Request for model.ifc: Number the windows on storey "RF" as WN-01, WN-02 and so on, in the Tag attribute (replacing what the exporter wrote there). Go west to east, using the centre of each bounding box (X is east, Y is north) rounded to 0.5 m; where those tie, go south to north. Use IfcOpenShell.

First a look at what the model holds.

```python
import ifcopenshell
import ifcopenshell.util.element
import ifcopenshell.util.placement

model = ifcopenshell.open("model.ifc")
print(model.schema)
storey = next(s for s in model.by_type("IfcBuildingStorey") if s.Name == "RF")
windows = [e for e in ifcopenshell.util.element.get_decomposition(storey) if e.is_a("IfcWindow")]
for e in sorted(windows, key=lambda e: e.id()):
    origin = ifcopenshell.util.placement.get_local_placement(e.ObjectPlacement)[:3, 3]
    print(e.id(), e.Tag, e.Name, origin.round(2) + 0.0, sep=" | ")
```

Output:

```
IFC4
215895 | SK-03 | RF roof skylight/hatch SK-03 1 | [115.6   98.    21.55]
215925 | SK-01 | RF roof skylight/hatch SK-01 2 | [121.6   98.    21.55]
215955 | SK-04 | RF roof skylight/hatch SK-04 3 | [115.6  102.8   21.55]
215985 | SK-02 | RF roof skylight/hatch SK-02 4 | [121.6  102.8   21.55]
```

```python
import ifcopenshell
import ifcopenshell.geom
import ifcopenshell.util.element
import ifcopenshell.util.shape

model = ifcopenshell.open("model.ifc")
settings = ifcopenshell.geom.settings()
settings.set("use-world-coords", True)


def centre(element):
    shape = ifcopenshell.geom.create_shape(settings, element)
    return ifcopenshell.util.shape.get_bbox_centroid(shape.geometry)


storey = next(s for s in model.by_type("IfcBuildingStorey") if s.Name == "RF")
windows = [e for e in ifcopenshell.util.element.get_decomposition(storey) if e.is_a("IfcWindow")]

# Insertion points can sit at a corner or the storey origin, so sort by the geometry (in metres).
centres = {e: centre(e) for e in windows}
windows.sort(key=lambda e: (round(centres[e][0] / 0.5), centres[e][1]))

for i, e in enumerate(windows, start=1):
    number = f"WN-{i:02d}"
    e.Tag = number
    print(e.id(), number)

model.write("model_v2.ifc")
```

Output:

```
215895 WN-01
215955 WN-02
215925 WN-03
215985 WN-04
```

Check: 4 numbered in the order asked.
